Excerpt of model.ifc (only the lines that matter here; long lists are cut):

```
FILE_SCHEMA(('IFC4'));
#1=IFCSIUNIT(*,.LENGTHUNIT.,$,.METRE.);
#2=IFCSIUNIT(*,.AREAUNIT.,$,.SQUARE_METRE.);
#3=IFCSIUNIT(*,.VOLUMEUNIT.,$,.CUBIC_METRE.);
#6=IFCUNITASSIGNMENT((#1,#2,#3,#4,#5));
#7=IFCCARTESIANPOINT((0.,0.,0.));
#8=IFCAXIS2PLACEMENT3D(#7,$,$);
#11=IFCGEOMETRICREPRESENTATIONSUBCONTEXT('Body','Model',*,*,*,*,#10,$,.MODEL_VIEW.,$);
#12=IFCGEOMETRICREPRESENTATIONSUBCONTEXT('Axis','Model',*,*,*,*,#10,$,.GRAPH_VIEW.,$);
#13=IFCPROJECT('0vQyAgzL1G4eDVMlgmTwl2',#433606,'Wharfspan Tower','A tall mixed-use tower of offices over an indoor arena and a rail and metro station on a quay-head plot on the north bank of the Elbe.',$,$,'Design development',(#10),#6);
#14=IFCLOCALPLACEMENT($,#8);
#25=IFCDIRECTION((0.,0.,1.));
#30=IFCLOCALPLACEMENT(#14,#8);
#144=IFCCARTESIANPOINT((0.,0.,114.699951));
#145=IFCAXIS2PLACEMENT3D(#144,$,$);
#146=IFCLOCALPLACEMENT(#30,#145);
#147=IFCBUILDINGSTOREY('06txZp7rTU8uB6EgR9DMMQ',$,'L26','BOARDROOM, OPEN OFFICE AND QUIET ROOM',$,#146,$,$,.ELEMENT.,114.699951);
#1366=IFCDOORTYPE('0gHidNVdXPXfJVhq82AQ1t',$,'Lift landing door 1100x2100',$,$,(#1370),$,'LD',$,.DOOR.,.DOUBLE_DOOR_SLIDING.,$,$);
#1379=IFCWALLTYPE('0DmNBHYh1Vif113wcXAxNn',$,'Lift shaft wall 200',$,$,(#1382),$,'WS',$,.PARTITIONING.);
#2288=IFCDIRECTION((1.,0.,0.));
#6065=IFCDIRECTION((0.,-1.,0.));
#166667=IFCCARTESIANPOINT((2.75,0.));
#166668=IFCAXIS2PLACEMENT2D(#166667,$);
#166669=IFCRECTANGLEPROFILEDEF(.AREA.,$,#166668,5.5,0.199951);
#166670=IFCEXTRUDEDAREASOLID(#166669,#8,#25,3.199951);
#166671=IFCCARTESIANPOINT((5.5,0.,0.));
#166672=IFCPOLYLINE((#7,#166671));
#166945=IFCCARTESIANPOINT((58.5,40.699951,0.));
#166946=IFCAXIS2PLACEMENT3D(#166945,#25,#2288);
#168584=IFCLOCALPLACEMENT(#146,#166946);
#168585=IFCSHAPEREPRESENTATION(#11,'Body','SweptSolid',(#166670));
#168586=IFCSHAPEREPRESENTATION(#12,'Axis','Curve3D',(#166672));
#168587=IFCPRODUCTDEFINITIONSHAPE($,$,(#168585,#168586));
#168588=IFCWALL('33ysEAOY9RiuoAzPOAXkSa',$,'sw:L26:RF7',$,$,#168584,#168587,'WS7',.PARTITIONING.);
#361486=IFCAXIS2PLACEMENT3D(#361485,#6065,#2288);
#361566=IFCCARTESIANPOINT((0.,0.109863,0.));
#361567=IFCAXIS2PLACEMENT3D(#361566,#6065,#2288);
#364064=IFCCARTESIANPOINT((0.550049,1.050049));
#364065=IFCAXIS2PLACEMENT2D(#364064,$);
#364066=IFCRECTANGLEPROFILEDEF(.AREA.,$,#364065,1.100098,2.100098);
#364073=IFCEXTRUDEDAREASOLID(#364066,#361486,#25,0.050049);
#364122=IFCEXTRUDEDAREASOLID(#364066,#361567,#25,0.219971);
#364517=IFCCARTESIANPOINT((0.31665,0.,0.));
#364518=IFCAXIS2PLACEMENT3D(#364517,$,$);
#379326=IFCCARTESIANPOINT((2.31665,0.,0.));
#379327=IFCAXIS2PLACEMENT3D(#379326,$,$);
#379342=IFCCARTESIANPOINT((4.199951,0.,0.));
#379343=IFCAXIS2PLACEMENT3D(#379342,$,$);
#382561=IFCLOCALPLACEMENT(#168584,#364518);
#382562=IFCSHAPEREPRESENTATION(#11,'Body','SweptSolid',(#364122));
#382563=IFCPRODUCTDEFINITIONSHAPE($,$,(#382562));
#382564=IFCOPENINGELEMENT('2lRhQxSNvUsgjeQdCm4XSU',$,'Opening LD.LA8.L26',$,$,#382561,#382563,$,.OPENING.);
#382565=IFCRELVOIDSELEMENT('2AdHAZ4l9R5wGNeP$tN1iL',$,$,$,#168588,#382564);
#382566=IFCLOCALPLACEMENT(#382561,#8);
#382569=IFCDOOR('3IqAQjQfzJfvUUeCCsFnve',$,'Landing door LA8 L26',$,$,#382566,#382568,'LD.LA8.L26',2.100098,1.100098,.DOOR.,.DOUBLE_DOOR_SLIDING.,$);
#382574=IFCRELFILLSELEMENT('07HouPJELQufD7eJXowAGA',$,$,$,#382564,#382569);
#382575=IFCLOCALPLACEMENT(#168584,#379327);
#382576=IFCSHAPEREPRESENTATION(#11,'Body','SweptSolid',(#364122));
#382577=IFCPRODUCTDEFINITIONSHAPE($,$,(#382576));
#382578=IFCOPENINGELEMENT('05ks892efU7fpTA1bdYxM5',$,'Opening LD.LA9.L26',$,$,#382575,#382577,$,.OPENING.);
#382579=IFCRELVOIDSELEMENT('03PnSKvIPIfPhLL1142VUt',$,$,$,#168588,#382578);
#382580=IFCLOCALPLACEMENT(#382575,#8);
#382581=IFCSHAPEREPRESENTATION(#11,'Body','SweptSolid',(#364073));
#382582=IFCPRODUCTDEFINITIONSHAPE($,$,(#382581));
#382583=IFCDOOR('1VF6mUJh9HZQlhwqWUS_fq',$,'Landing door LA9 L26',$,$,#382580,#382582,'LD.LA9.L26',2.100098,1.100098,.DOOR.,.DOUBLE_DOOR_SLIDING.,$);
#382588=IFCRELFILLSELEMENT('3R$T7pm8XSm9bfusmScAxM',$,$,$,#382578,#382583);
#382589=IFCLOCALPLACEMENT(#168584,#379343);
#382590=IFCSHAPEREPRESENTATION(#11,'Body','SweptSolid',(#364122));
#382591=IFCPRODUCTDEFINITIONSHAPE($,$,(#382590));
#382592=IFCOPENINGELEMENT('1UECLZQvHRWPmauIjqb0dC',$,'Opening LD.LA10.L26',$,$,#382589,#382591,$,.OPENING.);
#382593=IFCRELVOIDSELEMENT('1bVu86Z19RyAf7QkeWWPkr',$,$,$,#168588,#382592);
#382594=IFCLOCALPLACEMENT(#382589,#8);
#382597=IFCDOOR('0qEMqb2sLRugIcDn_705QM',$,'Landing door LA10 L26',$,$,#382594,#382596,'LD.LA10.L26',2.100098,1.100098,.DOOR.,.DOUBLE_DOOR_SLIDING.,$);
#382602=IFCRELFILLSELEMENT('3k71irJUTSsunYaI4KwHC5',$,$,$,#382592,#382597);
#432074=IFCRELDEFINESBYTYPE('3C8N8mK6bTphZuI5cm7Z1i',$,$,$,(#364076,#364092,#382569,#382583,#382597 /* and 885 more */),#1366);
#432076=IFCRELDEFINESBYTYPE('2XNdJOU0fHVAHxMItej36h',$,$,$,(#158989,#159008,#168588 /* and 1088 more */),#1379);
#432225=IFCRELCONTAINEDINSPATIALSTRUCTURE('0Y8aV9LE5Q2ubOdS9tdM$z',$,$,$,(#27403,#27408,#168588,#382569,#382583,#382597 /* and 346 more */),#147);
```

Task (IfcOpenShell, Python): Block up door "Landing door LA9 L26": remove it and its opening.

```python
import ifcopenshell
import ifcopenshell.api.feature
import ifcopenshell.api.root
import ifcopenshell.geom
import ifcopenshell.util.shape

model = ifcopenshell.open("model.ifc")
settings = ifcopenshell.geom.settings()


def volume(element):
    """Net volume in cubic metres, openings subtracted."""
    shape = ifcopenshell.geom.create_shape(settings, element)
    return ifcopenshell.util.shape.get_volume(shape.geometry)


door = model.by_guid("1VF6mUJh9HZQlhwqWUS_fq")
opening = door.FillsVoids[0].RelatingOpeningElement
wall = opening.VoidsElements[0].RelatingBuildingElement
before = volume(wall)

ifcopenshell.api.root.remove_product(model, product=door)
ifcopenshell.api.feature.remove_feature(model, feature=opening)

after = volume(wall)

print(f"wall volume {before:.3f} -> {after:.3f} m3")

model.write("model_rev.ifc")
```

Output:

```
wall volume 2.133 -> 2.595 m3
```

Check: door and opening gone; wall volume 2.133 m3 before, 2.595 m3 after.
